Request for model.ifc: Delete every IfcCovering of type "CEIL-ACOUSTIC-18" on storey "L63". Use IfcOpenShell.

First a look at what the model holds.

```python
import ifcopenshell
import ifcopenshell.util.element

model = ifcopenshell.open("model.ifc")
print(model.schema)
storey = next(s for s in model.by_type("IfcBuildingStorey") if s.Name == "L63")
coverings = [e for e in ifcopenshell.util.element.get_decomposition(storey) if e.is_a("IfcCovering")]
seen = {}
for e in coverings:
    element_type = ifcopenshell.util.element.get_type(e)
    name = element_type.Name if element_type not in (None, e) else None
    seen[name] = seen.get(name, 0) + 1
for name, count in sorted(seen.items(), key=str):
    print(count, "x", name)
```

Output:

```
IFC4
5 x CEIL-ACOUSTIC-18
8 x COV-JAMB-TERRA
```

```python
import ifcopenshell
import ifcopenshell.api.root
import ifcopenshell.util.element

model = ifcopenshell.open("model.ifc")

storey = next(s for s in model.by_type("IfcBuildingStorey") if s.Name == "L63")
coverings = [e for e in ifcopenshell.util.element.get_decomposition(storey) if e.is_a("IfcCovering")]
targets = [e for e in coverings if (t := ifcopenshell.util.element.get_type(e)) not in (None, e) and t.Name == "CEIL-ACOUSTIC-18"]

for e in targets:
    ifcopenshell.api.root.remove_product(model, product=e)
print(len(targets), "removed")

model.write("model_updated.ifc")
```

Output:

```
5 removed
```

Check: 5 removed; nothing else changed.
